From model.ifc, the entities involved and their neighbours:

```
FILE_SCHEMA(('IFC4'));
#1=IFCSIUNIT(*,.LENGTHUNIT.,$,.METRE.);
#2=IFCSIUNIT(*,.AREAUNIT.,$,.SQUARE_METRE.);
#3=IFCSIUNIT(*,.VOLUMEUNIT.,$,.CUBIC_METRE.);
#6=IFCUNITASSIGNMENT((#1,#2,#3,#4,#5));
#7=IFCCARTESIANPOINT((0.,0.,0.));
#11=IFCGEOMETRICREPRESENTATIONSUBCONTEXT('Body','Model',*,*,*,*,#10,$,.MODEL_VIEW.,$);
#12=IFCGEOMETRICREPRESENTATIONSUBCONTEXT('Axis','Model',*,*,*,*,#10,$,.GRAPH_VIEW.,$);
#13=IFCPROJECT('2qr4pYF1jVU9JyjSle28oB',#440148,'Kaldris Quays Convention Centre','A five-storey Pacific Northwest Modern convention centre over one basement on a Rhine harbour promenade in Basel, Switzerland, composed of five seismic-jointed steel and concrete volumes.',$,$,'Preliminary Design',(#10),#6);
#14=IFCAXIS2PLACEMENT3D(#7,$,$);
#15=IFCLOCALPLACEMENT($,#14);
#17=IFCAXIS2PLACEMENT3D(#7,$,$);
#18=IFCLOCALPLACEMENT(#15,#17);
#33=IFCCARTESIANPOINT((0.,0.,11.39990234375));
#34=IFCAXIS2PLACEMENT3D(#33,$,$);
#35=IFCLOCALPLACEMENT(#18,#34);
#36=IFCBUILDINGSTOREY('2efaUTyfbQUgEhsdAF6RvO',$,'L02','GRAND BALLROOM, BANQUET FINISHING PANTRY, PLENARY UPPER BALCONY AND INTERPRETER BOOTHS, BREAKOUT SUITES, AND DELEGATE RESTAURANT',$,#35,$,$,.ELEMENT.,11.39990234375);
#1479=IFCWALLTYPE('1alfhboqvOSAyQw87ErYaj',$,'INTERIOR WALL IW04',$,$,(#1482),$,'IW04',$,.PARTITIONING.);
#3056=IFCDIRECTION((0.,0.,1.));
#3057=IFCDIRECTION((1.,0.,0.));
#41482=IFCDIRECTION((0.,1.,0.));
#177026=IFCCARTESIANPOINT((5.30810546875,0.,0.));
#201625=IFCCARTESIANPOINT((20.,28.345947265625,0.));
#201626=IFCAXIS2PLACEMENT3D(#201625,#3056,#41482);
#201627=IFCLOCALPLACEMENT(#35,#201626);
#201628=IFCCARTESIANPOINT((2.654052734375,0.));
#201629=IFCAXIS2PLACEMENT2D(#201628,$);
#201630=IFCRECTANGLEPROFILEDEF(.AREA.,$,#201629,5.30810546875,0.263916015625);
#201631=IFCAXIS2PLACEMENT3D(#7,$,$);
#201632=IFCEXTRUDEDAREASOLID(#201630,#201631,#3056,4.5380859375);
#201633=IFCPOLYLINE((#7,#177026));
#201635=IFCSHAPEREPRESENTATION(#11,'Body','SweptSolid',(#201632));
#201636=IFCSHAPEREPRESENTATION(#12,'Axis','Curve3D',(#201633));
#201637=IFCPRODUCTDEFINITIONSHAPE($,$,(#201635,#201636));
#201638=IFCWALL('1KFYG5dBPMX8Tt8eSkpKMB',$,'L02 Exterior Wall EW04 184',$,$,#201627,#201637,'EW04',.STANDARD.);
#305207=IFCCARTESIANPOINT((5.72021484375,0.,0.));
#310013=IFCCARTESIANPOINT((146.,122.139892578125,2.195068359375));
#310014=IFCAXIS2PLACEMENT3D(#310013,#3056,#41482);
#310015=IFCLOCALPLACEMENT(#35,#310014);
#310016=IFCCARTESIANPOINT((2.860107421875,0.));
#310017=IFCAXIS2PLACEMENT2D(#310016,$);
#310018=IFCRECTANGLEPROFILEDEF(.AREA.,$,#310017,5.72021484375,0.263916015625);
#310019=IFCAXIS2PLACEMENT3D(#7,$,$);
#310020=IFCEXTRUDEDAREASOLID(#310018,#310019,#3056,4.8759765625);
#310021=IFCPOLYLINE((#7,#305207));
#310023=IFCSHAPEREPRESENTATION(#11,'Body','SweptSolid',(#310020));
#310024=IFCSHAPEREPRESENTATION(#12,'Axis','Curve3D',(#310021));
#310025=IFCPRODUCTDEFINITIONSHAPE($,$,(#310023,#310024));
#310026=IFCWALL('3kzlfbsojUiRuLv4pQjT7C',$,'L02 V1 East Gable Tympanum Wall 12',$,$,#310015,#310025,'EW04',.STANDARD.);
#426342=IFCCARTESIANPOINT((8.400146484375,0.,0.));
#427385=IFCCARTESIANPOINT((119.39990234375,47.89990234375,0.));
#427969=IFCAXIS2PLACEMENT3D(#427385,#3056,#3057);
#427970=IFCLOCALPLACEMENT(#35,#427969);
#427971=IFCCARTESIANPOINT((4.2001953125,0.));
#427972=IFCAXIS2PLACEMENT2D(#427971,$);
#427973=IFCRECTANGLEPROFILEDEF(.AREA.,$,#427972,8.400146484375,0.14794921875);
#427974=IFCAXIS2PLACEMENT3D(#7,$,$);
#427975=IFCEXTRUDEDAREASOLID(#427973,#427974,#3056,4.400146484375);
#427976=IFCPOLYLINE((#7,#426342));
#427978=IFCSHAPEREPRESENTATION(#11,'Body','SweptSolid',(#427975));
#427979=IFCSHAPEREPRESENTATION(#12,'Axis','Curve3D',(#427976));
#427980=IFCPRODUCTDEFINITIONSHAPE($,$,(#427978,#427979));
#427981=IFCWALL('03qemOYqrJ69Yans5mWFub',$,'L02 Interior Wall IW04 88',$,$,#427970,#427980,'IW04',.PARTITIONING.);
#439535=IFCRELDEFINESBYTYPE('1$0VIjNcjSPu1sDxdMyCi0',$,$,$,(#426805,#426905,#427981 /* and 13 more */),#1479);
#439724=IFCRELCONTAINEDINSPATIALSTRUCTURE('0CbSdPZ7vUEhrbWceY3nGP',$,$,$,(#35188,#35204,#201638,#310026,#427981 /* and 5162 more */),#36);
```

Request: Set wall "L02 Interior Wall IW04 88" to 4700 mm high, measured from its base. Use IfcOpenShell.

```python
import ifcopenshell
import ifcopenshell.geom
import ifcopenshell.util.representation
import ifcopenshell.util.shape

model = ifcopenshell.open("model.ifc")
settings = ifcopenshell.geom.settings()


def volume(element):
    """Net volume in cubic metres, openings subtracted."""
    shape = ifcopenshell.geom.create_shape(settings, element)
    return ifcopenshell.util.shape.get_volume(shape.geometry)


wall = model.by_guid("03qemOYqrJ69Yans5mWFub")
before = volume(wall)

body = ifcopenshell.util.representation.get_representation(wall, "Model", "Body")
solid = body.Items[0]
old_height = solid.Depth
solid.Depth = 4.7
after = volume(wall)

print(f"height {old_height:g} -> {solid.Depth:g}, volume {before:.3f} -> {after:.3f} m3")

model.write("model_v2.ifc")
```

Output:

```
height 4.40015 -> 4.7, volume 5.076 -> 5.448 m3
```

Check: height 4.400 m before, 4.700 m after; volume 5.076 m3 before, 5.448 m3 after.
